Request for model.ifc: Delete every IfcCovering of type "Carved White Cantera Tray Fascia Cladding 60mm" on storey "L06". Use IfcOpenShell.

First a look at what the model holds.

```python
import ifcopenshell
import ifcopenshell.util.element

model = ifcopenshell.open("model.ifc")
print(model.schema)
storey = next(s for s in model.by_type("IfcBuildingStorey") if s.Name == "L06")
coverings = [e for e in ifcopenshell.util.element.get_decomposition(storey) if e.is_a("IfcCovering")]
seen = {}
for e in coverings:
    element_type = ifcopenshell.util.element.get_type(e)
    name = element_type.Name if element_type not in (None, e) else None
    seen[name] = seen.get(name, 0) + 1
for name, count in sorted(seen.items(), key=str):
    print(count, "x", name)
```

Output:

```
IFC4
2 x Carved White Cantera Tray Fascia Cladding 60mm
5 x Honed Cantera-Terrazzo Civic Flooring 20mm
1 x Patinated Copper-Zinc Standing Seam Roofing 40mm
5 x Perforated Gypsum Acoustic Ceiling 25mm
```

```python
import ifcopenshell
import ifcopenshell.api.root
import ifcopenshell.util.element

model = ifcopenshell.open("model.ifc")

storey = next(s for s in model.by_type("IfcBuildingStorey") if s.Name == "L06")
coverings = [e for e in ifcopenshell.util.element.get_decomposition(storey) if e.is_a("IfcCovering")]
targets = [e for e in coverings if (t := ifcopenshell.util.element.get_type(e)) not in (None, e) and t.Name == "Carved White Cantera Tray Fascia Cladding 60mm"]

for e in targets:
    ifcopenshell.api.root.remove_product(model, product=e)
print(len(targets), "removed")

model.write("model_updated.ifc")
```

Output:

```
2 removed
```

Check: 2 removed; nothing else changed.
